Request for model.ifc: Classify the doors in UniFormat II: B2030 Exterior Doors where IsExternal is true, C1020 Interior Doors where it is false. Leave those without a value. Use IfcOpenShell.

First a look at what the model holds.

```python
import ifcopenshell
import ifcopenshell.util.element

model = ifcopenshell.open("model.ifc")
print(model.schema)
print("classifications:", [c.Name for c in model.by_type("IfcClassification")])
values = [ifcopenshell.util.element.get_pset(e, "Pset_DoorCommon", "IsExternal") for e in model.by_type("IfcDoor")]
for value in (True, False, None):
    print("IsExternal", value, values.count(value))
```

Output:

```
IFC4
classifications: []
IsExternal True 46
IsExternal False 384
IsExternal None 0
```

```python
import ifcopenshell
import ifcopenshell.api.classification
import ifcopenshell.util.element

model = ifcopenshell.open("model.ifc")

system = ifcopenshell.api.classification.add_classification(model, classification="UniFormat II")

doors = model.by_type("IfcDoor")
external = {e: ifcopenshell.util.element.get_pset(e, "Pset_DoorCommon", "IsExternal") for e in doors}
for flag, code, name in ((True, "B2030", "Exterior Doors"), (False, "C1020", "Interior Doors")):
    products = [e for e in doors if external[e] is flag]
    ifcopenshell.api.classification.add_reference(
        model, products=products, classification=system, identification=code, name=name
    )
    print(code, len(products))

model.write("model_v2.ifc")
```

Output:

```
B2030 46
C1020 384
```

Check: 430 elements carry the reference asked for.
